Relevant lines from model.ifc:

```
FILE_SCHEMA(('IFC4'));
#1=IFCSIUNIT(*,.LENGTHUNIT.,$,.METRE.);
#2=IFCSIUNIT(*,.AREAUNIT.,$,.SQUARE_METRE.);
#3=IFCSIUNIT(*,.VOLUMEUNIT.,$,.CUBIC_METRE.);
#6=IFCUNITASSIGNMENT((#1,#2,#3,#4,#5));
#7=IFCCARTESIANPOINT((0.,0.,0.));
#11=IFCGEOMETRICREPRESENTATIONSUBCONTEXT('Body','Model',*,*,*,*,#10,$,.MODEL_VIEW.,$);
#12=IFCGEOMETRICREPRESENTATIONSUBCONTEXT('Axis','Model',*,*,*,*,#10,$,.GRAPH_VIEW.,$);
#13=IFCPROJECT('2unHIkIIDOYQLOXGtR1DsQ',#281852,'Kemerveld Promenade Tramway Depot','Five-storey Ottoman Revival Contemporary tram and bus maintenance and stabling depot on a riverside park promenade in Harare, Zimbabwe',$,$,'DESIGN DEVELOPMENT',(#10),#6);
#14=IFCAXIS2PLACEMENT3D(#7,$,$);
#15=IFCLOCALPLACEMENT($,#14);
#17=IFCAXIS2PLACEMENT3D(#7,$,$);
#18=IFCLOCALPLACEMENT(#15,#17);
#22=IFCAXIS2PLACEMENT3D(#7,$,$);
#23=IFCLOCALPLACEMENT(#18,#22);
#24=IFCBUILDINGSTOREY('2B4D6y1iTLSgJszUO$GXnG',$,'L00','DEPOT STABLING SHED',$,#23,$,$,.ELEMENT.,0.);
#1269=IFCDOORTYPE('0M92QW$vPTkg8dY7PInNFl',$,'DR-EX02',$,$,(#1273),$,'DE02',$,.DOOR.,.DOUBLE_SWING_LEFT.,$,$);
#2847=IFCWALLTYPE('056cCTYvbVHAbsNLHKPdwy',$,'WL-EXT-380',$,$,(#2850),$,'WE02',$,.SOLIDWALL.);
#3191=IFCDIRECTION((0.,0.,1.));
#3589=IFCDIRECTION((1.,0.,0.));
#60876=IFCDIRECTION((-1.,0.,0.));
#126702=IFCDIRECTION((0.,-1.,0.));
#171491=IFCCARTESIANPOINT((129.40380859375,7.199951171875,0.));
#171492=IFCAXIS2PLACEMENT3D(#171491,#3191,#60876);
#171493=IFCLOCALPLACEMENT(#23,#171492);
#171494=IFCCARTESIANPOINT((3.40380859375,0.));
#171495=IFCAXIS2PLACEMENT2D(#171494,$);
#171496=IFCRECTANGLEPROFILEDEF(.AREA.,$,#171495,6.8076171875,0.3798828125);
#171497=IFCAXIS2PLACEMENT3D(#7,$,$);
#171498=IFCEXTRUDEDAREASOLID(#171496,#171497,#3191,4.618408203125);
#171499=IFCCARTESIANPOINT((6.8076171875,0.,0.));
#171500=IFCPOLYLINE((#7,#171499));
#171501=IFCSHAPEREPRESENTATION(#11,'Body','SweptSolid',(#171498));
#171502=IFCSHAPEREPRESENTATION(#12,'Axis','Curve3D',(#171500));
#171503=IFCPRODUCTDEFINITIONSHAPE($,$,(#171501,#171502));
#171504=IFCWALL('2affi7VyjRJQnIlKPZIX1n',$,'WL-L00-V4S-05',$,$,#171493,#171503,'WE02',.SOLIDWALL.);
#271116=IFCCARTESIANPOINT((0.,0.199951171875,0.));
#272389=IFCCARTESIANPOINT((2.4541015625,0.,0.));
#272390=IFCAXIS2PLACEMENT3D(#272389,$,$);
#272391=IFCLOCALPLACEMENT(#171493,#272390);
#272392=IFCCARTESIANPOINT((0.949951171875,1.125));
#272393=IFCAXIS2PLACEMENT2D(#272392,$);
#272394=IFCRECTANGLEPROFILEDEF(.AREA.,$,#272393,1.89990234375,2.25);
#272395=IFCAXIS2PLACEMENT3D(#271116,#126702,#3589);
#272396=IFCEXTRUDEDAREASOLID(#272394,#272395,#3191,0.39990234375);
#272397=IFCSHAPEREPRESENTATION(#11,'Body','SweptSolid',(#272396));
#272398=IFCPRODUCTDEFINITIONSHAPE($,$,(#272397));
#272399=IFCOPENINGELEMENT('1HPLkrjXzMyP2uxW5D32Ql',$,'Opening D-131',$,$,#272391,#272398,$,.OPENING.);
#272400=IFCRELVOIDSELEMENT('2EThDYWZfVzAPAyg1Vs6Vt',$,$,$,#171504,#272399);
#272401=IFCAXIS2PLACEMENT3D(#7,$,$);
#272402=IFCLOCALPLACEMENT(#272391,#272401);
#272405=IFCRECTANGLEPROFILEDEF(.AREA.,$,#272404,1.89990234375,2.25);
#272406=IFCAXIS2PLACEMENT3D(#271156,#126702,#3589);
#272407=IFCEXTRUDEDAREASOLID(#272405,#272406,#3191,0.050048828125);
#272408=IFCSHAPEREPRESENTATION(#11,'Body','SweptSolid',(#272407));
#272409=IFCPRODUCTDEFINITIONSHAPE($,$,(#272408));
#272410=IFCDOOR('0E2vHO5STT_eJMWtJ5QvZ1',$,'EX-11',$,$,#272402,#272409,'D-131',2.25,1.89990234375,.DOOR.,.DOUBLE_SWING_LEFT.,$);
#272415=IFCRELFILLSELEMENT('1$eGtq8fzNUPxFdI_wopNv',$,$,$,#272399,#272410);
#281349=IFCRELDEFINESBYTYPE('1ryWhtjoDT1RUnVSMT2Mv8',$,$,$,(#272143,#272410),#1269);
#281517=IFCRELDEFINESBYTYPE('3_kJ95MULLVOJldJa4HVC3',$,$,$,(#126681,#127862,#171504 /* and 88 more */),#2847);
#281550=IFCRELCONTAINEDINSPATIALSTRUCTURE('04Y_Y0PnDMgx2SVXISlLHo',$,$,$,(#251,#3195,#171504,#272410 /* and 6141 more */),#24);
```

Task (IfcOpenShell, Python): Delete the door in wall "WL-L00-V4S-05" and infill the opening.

```python
import ifcopenshell
import ifcopenshell.api.feature
import ifcopenshell.api.root
import ifcopenshell.geom
import ifcopenshell.util.shape

model = ifcopenshell.open("model.ifc")
settings = ifcopenshell.geom.settings()


def volume(element):
    """Net volume in cubic metres, openings subtracted."""
    shape = ifcopenshell.geom.create_shape(settings, element)
    return ifcopenshell.util.shape.get_volume(shape.geometry)


door = model.by_guid("0E2vHO5STT_eJMWtJ5QvZ1")
opening = door.FillsVoids[0].RelatingOpeningElement
wall = opening.VoidsElements[0].RelatingBuildingElement
before = volume(wall)

ifcopenshell.api.root.remove_product(model, product=door)
ifcopenshell.api.feature.remove_feature(model, feature=opening)

after = volume(wall)

print(f"wall volume {before:.3f} -> {after:.3f} m3")

model.write("model-out.ifc")
```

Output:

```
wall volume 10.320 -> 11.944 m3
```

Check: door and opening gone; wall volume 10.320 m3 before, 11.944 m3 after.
